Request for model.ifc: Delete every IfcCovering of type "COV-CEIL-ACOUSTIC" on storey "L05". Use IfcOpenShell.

First a look at what the model holds.

```python
import ifcopenshell
import ifcopenshell.util.element

model = ifcopenshell.open("model.ifc")
print(model.schema)
storey = next(s for s in model.by_type("IfcBuildingStorey") if s.Name == "L05")
coverings = [e for e in ifcopenshell.util.element.get_decomposition(storey) if e.is_a("IfcCovering")]
seen = {}
for e in coverings:
    element_type = ifcopenshell.util.element.get_type(e)
    name = element_type.Name if element_type not in (None, e) else None
    seen[name] = seen.get(name, 0) + 1
for name, count in sorted(seen.items(), key=str):
    print(count, "x", name)
```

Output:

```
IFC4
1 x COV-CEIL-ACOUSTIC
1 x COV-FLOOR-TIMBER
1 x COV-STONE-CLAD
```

```python
import ifcopenshell
import ifcopenshell.api.root
import ifcopenshell.util.element

model = ifcopenshell.open("model.ifc")

storey = next(s for s in model.by_type("IfcBuildingStorey") if s.Name == "L05")
coverings = [e for e in ifcopenshell.util.element.get_decomposition(storey) if e.is_a("IfcCovering")]
targets = [e for e in coverings if (t := ifcopenshell.util.element.get_type(e)) not in (None, e) and t.Name == "COV-CEIL-ACOUSTIC"]

for e in targets:
    ifcopenshell.api.root.remove_product(model, product=e)
print(len(targets), "removed")

model.write("model_v2.ifc")
```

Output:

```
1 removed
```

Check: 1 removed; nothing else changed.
